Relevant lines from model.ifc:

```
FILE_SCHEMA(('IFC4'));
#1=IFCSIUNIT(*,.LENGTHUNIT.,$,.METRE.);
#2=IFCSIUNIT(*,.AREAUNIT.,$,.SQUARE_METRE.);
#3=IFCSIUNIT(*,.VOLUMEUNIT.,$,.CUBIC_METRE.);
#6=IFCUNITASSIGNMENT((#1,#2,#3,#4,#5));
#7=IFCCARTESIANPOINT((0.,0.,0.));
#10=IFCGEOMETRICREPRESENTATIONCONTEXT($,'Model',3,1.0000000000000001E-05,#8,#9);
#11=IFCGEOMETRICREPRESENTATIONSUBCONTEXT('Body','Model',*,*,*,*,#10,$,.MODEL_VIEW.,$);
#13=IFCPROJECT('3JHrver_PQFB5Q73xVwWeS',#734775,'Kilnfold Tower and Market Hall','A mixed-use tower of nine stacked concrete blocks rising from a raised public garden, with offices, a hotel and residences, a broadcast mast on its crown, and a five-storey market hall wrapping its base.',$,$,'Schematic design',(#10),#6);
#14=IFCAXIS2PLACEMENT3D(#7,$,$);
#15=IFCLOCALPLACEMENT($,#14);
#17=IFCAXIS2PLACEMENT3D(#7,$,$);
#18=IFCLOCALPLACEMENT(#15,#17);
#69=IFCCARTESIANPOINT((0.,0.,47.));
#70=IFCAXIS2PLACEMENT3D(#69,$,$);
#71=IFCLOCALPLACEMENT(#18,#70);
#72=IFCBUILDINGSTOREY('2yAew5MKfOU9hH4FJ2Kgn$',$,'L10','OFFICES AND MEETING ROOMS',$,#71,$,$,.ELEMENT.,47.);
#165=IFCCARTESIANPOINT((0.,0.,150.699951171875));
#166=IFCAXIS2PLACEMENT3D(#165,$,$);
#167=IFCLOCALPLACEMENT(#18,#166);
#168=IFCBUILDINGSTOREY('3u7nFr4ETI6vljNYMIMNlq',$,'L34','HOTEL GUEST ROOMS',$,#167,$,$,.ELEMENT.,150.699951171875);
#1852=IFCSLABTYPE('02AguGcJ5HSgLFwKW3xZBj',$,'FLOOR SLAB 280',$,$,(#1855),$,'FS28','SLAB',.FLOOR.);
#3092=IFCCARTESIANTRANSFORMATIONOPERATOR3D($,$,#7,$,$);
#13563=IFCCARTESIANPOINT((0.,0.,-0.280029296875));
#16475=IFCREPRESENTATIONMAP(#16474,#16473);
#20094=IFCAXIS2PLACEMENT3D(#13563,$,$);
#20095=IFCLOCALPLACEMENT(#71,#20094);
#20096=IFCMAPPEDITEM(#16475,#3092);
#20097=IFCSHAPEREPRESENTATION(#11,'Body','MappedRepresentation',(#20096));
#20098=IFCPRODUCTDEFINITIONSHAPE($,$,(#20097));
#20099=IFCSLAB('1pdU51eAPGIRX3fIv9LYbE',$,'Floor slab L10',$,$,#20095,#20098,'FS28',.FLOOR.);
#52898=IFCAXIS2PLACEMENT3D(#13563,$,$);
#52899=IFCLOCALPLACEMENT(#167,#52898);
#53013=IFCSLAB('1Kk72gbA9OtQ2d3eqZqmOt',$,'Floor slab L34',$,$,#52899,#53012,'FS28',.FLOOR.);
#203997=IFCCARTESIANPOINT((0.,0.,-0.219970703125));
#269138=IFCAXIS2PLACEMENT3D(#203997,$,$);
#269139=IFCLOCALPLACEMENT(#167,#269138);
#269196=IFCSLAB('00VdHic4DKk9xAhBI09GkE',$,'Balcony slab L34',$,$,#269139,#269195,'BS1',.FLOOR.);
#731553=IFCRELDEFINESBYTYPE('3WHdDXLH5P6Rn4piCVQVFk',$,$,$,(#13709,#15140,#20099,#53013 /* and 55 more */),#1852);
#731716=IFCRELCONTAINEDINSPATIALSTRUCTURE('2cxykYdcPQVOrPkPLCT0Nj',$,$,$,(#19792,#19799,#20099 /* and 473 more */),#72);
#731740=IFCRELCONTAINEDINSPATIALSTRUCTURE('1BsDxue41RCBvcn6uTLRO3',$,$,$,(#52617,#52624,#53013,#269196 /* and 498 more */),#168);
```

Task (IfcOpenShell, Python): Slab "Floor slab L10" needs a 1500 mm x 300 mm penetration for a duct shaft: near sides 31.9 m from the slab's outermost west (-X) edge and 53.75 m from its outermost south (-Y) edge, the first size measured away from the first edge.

```python
import numpy as np
import ifcopenshell
import ifcopenshell.api.feature
import ifcopenshell.api.geometry
import ifcopenshell.api.root
import ifcopenshell.geom
import ifcopenshell.util.placement
import ifcopenshell.util.representation
import ifcopenshell.util.shape
import ifcopenshell.util.unit

model = ifcopenshell.open("model.ifc")
unit_scale = ifcopenshell.util.unit.calculate_unit_scale(model)
settings = ifcopenshell.geom.settings()


def volume(element):
    """Net volume in cubic metres, openings subtracted."""
    shape = ifcopenshell.geom.create_shape(settings, element)
    return ifcopenshell.util.shape.get_volume(shape.geometry)


slab = model.by_guid("1pdU51eAPGIRX3fIv9LYbE")
before = volume(slab)

# Extent in the slab's own axes, in metres. The edges named are its -X and -Y sides.
slab_shape = ifcopenshell.geom.create_shape(settings, slab)
vertices = ifcopenshell.util.shape.get_vertices(slab_shape.geometry)
x_min, y_min, bottom = vertices.min(axis=0)
top = vertices[:, 2].max()

opening = ifcopenshell.api.root.create_entity(model, ifc_class="IfcOpeningElement", name="Duct shaft opening", predefined_type="OPENING")
context = ifcopenshell.util.representation.get_context(model, "Model", "Body", "MODEL_VIEW")
width, depth = 1.5, 0.3
outline = [(0.0, 0.0), (width, 0.0), (width, depth), (0.0, depth), (0.0, 0.0)]
# Overshoot both faces by 50 mm so the cut is clean.
shape = ifcopenshell.api.geometry.add_slab_representation(
    model, context=context, depth=top - bottom + 0.1, polyline=outline
)
ifcopenshell.api.geometry.assign_representation(model, product=opening, representation=shape)

matrix = ifcopenshell.util.placement.get_local_placement(slab.ObjectPlacement)
matrix[:, 3] = matrix @ np.append(np.array([x_min + 31.9, y_min + 53.75, bottom - 0.05]) / unit_scale, 1.0)
ifcopenshell.api.geometry.edit_object_placement(model, product=opening, matrix=matrix, is_si=False)
ifcopenshell.api.feature.add_feature(model, feature=opening, element=slab)

after = volume(slab)

print(f"slab volume {before:.3f} -> {after:.3f} m3")

model.write("model_updated.ifc")
```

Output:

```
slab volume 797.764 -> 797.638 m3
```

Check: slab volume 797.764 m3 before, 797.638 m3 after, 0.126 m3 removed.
